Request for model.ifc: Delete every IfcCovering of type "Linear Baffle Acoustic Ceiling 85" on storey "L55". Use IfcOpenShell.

First a look at what the model holds.

```python
import ifcopenshell
import ifcopenshell.util.element

model = ifcopenshell.open("model.ifc")
print(model.schema)
storey = next(s for s in model.by_type("IfcBuildingStorey") if s.Name == "L55")
coverings = [e for e in ifcopenshell.util.element.get_decomposition(storey) if e.is_a("IfcCovering")]
seen = {}
for e in coverings:
    element_type = ifcopenshell.util.element.get_type(e)
    name = element_type.Name if element_type not in (None, e) else None
    seen[name] = seen.get(name, 0) + 1
for name, count in sorted(seen.items(), key=str):
    print(count, "x", name)
```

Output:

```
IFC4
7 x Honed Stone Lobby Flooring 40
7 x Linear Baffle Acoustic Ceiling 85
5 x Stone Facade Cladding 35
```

```python
import ifcopenshell
import ifcopenshell.api.root
import ifcopenshell.util.element

model = ifcopenshell.open("model.ifc")

storey = next(s for s in model.by_type("IfcBuildingStorey") if s.Name == "L55")
coverings = [e for e in ifcopenshell.util.element.get_decomposition(storey) if e.is_a("IfcCovering")]
targets = [e for e in coverings if (t := ifcopenshell.util.element.get_type(e)) not in (None, e) and t.Name == "Linear Baffle Acoustic Ceiling 85"]

for e in targets:
    ifcopenshell.api.root.remove_product(model, product=e)
print(len(targets), "removed")

model.write("model-out.ifc")
```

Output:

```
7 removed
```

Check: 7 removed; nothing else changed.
